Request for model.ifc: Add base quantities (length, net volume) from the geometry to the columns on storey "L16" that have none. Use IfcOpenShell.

First a look at what the model holds.

```python
import ifcopenshell
import ifcopenshell.util.element
import ifcopenshell.util.unit

model = ifcopenshell.open("model.ifc")
print(model.schema)
for unit_type in ("LENGTHUNIT", "AREAUNIT", "VOLUMEUNIT"):
    print(unit_type, ifcopenshell.util.unit.calculate_unit_scale(model, unit_type))
storey = next(s for s in model.by_type("IfcBuildingStorey") if s.Name == "L16")
columns = [e for e in ifcopenshell.util.element.get_decomposition(storey) if e.is_a("IfcColumn")]
for e in sorted(columns, key=lambda e: e.id()):
    print(e.id(), e.is_a(), e.Name, list(ifcopenshell.util.element.get_psets(e, qtos_only=True)), sep=" | ")
```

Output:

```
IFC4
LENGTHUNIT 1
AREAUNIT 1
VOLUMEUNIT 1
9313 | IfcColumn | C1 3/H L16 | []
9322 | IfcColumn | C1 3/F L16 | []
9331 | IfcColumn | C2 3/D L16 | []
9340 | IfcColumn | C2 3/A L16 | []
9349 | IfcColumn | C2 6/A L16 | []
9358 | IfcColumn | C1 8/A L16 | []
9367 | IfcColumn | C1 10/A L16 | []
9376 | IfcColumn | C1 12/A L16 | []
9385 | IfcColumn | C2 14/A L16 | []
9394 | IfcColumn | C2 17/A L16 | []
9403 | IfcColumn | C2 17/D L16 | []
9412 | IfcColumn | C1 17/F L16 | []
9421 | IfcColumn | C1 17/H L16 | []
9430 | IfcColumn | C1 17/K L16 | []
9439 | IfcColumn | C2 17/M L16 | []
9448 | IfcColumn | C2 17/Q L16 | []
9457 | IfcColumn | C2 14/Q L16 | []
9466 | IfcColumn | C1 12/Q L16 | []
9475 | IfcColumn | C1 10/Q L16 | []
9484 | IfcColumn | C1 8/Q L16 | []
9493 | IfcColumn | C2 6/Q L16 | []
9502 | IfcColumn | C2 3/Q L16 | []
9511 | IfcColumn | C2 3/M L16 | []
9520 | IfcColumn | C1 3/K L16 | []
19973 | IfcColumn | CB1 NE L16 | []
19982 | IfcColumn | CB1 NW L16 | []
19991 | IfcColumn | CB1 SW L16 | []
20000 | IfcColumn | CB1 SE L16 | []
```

```python
import ifcopenshell
import ifcopenshell.api.pset
import ifcopenshell.geom
import ifcopenshell.util.element
import ifcopenshell.util.shape
import ifcopenshell.util.unit

model = ifcopenshell.open("model.ifc")
unit_scale = ifcopenshell.util.unit.calculate_unit_scale(model)
volume_scale = ifcopenshell.util.unit.calculate_unit_scale(model, "VOLUMEUNIT")
settings = ifcopenshell.geom.settings()

storey = next(s for s in model.by_type("IfcBuildingStorey") if s.Name == "L16")
columns = [e for e in ifcopenshell.util.element.get_decomposition(storey) if e.is_a("IfcColumn")]

for e in sorted(columns, key=lambda e: e.id()):
    if ifcopenshell.util.element.get_psets(e, qtos_only=True, should_inherit=False):
        continue
    # Geometry comes back in metres, in the element's own axes.
    shape = ifcopenshell.geom.create_shape(settings, e)
    values = {
        "Length": ifcopenshell.util.shape.get_z(shape.geometry) / unit_scale,
        "NetVolume": ifcopenshell.util.shape.get_volume(shape.geometry) / volume_scale,
    }
    qto = ifcopenshell.api.pset.add_qto(model, product=e, name="Qto_ColumnBaseQuantities")
    ifcopenshell.api.pset.edit_qto(model, qto=qto, properties=values)
    print(e.id(), {k: round(v, 3) for k, v in values.items()})

model.write("model_rev.ifc")
```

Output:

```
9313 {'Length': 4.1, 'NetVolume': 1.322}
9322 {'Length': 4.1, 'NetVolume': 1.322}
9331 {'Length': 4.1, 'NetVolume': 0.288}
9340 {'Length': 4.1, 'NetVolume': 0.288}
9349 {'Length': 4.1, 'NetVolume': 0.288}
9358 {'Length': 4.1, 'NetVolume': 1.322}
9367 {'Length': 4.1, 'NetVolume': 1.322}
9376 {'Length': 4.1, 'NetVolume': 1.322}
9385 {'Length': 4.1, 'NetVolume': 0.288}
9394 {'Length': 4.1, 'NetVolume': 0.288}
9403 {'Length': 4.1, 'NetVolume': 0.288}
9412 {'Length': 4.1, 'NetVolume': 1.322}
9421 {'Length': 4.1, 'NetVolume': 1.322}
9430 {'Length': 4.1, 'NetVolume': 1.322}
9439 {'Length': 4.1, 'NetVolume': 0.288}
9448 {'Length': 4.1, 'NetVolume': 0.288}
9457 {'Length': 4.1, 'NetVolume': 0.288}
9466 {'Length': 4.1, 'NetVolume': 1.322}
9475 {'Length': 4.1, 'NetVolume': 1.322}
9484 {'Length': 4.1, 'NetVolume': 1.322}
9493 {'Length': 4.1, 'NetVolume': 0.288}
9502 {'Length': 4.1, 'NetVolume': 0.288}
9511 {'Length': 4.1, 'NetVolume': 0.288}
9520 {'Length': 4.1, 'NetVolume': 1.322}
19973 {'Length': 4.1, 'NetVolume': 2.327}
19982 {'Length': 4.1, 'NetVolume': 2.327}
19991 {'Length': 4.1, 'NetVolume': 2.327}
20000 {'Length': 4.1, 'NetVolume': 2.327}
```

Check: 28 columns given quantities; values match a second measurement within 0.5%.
